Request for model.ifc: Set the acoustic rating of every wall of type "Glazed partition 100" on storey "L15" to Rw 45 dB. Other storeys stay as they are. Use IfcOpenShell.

First a look at what the model holds.

```python
import ifcopenshell
import ifcopenshell.util.element

model = ifcopenshell.open("model.ifc")
print(model.schema)
storey = next(s for s in model.by_type("IfcBuildingStorey") if s.Name == "L15")
walls = [e for e in ifcopenshell.util.element.get_decomposition(storey) if e.is_a("IfcWall")]
seen = {}
for e in walls:
    element_type = ifcopenshell.util.element.get_type(e)
    key = (element_type.Name if element_type != e and element_type else None, ifcopenshell.util.element.get_pset(e, "Pset_WallCommon", "AcousticRating"))
    seen[key] = seen.get(key, 0) + 1
for (name, value), count in sorted(seen.items(), key=str):
    print(count, "x", name, "|", value)
```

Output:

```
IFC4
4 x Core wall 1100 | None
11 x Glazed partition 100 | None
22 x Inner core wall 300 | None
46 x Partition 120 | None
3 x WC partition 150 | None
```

```python
import ifcopenshell
import ifcopenshell.api.pset
import ifcopenshell.util.element

model = ifcopenshell.open("model.ifc")

storey = next(s for s in model.by_type("IfcBuildingStorey") if s.Name == "L15")
walls = [e for e in ifcopenshell.util.element.get_decomposition(storey) if e.is_a("IfcWall")]

count = 0
for e in walls:
    element_type = ifcopenshell.util.element.get_type(e)
    if element_type in (None, e) or element_type.Name != "Glazed partition 100":
        continue
    # add_pset returns the element's existing set when there is one.
    pset = ifcopenshell.api.pset.add_pset(model, product=e, name="Pset_WallCommon")
    ifcopenshell.api.pset.edit_pset(model, pset=pset, properties={"AcousticRating": "Rw 45 dB"})
    count += 1

print(count, "walls updated")

model.write("model_v2.ifc")
```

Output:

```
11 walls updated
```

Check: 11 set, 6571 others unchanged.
